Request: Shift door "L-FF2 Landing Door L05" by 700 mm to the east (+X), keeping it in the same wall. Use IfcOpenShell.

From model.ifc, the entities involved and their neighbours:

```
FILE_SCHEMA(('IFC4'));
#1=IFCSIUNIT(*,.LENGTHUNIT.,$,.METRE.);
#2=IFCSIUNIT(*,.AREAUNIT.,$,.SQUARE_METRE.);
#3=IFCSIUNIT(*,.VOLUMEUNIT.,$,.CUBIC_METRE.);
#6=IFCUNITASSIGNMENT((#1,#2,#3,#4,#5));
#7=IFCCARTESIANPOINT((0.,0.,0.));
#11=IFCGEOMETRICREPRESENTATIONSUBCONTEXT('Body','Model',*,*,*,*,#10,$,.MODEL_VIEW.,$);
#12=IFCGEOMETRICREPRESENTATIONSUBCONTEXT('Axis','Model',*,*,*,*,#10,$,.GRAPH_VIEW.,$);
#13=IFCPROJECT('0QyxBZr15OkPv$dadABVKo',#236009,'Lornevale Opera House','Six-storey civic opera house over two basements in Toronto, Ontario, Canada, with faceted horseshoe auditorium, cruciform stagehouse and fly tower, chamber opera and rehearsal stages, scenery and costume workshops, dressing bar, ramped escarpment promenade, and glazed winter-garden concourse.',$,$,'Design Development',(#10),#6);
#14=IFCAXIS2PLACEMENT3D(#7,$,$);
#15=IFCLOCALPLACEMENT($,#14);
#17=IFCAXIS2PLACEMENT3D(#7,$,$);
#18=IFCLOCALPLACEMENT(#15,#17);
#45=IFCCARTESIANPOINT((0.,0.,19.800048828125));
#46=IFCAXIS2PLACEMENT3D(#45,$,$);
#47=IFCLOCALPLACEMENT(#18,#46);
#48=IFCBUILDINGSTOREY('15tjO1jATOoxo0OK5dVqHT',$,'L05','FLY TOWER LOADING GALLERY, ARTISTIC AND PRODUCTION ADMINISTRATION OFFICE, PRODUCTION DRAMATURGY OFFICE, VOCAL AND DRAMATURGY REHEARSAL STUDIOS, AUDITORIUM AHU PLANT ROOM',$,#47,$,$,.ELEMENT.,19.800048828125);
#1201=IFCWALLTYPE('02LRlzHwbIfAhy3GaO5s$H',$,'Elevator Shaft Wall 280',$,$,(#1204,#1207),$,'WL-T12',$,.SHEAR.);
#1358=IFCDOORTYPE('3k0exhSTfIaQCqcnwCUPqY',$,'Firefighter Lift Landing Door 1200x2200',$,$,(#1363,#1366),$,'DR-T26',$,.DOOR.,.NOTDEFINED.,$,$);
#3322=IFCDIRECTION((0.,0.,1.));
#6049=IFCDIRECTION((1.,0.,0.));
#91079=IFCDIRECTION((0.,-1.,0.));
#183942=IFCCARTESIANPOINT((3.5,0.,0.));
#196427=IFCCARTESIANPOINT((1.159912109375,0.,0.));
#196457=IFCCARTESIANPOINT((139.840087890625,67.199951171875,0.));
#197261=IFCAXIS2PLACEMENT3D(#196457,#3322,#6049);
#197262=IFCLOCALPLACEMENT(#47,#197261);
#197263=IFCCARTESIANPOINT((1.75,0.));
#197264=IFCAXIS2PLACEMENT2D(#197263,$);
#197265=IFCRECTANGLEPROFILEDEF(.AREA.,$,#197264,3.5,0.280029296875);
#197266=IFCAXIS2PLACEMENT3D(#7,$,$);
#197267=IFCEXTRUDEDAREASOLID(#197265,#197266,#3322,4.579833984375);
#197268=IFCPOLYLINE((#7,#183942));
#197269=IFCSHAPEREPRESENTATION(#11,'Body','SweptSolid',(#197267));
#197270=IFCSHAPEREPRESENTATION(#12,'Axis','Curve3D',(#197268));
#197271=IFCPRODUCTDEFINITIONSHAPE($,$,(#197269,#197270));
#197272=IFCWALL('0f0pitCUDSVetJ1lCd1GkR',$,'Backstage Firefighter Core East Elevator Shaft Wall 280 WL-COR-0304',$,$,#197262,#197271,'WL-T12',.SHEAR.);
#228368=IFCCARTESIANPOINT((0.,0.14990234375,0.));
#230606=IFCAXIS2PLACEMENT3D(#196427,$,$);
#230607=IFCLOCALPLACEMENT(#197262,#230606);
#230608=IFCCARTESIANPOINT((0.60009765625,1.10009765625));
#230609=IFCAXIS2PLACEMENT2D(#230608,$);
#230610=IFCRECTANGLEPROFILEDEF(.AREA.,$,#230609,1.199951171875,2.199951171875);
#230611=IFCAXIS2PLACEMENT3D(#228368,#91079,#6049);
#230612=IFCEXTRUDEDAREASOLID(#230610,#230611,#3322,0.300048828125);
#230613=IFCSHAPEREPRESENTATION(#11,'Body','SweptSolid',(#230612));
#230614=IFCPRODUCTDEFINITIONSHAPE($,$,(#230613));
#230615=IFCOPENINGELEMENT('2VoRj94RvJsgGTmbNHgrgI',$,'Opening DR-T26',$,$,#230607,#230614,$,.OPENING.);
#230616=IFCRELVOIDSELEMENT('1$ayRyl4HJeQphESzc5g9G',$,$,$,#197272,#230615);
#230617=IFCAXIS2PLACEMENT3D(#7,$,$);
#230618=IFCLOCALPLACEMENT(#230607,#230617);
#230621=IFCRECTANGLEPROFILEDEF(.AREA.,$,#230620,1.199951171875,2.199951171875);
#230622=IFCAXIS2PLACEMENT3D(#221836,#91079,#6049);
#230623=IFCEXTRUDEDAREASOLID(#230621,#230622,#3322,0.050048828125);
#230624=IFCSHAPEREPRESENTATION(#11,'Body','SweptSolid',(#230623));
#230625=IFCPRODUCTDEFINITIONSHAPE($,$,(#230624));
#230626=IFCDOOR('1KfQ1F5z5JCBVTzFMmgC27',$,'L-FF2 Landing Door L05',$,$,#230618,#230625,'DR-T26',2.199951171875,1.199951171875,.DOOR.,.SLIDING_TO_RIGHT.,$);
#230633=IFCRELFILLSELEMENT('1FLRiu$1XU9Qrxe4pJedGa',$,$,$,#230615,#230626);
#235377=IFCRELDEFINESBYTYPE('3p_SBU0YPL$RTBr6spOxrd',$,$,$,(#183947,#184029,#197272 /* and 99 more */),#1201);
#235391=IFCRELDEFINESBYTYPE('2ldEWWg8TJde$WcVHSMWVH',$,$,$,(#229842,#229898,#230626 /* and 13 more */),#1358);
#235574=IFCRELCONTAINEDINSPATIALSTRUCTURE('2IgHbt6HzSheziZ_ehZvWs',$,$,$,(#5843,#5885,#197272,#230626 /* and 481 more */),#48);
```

```python
import ifcopenshell
import ifcopenshell.api.geometry
import ifcopenshell.util.placement
import ifcopenshell.util.unit

model = ifcopenshell.open("model.ifc")
unit_scale = ifcopenshell.util.unit.calculate_unit_scale(model)

door = model.by_guid("1KfQ1F5z5JCBVTzFMmgC27")
opening = door.FillsVoids[0].RelatingOpeningElement
wall = opening.VoidsElements[0].RelatingBuildingElement

wall_matrix = ifcopenshell.util.placement.get_local_placement(wall.ObjectPlacement)
shift = wall_matrix[:3, 0] * 0.7 / unit_scale
before = ifcopenshell.util.placement.get_local_placement(door.ObjectPlacement)[:3, 3].copy()

# The door is placed relative to its opening, so it follows when the opening moves.
matrix = ifcopenshell.util.placement.get_local_placement(opening.ObjectPlacement)
matrix[:3, 3] += shift
ifcopenshell.api.geometry.edit_object_placement(
    model, product=opening, matrix=matrix, is_si=False, should_transform_children=True
)

after = ifcopenshell.util.placement.get_local_placement(door.ObjectPlacement)[:3, 3]
print("door moved by", (after - before).round(3) + 0.0)

model.write("model_edited.ifc")
```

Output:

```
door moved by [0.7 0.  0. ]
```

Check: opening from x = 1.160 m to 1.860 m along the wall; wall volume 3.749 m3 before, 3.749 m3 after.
